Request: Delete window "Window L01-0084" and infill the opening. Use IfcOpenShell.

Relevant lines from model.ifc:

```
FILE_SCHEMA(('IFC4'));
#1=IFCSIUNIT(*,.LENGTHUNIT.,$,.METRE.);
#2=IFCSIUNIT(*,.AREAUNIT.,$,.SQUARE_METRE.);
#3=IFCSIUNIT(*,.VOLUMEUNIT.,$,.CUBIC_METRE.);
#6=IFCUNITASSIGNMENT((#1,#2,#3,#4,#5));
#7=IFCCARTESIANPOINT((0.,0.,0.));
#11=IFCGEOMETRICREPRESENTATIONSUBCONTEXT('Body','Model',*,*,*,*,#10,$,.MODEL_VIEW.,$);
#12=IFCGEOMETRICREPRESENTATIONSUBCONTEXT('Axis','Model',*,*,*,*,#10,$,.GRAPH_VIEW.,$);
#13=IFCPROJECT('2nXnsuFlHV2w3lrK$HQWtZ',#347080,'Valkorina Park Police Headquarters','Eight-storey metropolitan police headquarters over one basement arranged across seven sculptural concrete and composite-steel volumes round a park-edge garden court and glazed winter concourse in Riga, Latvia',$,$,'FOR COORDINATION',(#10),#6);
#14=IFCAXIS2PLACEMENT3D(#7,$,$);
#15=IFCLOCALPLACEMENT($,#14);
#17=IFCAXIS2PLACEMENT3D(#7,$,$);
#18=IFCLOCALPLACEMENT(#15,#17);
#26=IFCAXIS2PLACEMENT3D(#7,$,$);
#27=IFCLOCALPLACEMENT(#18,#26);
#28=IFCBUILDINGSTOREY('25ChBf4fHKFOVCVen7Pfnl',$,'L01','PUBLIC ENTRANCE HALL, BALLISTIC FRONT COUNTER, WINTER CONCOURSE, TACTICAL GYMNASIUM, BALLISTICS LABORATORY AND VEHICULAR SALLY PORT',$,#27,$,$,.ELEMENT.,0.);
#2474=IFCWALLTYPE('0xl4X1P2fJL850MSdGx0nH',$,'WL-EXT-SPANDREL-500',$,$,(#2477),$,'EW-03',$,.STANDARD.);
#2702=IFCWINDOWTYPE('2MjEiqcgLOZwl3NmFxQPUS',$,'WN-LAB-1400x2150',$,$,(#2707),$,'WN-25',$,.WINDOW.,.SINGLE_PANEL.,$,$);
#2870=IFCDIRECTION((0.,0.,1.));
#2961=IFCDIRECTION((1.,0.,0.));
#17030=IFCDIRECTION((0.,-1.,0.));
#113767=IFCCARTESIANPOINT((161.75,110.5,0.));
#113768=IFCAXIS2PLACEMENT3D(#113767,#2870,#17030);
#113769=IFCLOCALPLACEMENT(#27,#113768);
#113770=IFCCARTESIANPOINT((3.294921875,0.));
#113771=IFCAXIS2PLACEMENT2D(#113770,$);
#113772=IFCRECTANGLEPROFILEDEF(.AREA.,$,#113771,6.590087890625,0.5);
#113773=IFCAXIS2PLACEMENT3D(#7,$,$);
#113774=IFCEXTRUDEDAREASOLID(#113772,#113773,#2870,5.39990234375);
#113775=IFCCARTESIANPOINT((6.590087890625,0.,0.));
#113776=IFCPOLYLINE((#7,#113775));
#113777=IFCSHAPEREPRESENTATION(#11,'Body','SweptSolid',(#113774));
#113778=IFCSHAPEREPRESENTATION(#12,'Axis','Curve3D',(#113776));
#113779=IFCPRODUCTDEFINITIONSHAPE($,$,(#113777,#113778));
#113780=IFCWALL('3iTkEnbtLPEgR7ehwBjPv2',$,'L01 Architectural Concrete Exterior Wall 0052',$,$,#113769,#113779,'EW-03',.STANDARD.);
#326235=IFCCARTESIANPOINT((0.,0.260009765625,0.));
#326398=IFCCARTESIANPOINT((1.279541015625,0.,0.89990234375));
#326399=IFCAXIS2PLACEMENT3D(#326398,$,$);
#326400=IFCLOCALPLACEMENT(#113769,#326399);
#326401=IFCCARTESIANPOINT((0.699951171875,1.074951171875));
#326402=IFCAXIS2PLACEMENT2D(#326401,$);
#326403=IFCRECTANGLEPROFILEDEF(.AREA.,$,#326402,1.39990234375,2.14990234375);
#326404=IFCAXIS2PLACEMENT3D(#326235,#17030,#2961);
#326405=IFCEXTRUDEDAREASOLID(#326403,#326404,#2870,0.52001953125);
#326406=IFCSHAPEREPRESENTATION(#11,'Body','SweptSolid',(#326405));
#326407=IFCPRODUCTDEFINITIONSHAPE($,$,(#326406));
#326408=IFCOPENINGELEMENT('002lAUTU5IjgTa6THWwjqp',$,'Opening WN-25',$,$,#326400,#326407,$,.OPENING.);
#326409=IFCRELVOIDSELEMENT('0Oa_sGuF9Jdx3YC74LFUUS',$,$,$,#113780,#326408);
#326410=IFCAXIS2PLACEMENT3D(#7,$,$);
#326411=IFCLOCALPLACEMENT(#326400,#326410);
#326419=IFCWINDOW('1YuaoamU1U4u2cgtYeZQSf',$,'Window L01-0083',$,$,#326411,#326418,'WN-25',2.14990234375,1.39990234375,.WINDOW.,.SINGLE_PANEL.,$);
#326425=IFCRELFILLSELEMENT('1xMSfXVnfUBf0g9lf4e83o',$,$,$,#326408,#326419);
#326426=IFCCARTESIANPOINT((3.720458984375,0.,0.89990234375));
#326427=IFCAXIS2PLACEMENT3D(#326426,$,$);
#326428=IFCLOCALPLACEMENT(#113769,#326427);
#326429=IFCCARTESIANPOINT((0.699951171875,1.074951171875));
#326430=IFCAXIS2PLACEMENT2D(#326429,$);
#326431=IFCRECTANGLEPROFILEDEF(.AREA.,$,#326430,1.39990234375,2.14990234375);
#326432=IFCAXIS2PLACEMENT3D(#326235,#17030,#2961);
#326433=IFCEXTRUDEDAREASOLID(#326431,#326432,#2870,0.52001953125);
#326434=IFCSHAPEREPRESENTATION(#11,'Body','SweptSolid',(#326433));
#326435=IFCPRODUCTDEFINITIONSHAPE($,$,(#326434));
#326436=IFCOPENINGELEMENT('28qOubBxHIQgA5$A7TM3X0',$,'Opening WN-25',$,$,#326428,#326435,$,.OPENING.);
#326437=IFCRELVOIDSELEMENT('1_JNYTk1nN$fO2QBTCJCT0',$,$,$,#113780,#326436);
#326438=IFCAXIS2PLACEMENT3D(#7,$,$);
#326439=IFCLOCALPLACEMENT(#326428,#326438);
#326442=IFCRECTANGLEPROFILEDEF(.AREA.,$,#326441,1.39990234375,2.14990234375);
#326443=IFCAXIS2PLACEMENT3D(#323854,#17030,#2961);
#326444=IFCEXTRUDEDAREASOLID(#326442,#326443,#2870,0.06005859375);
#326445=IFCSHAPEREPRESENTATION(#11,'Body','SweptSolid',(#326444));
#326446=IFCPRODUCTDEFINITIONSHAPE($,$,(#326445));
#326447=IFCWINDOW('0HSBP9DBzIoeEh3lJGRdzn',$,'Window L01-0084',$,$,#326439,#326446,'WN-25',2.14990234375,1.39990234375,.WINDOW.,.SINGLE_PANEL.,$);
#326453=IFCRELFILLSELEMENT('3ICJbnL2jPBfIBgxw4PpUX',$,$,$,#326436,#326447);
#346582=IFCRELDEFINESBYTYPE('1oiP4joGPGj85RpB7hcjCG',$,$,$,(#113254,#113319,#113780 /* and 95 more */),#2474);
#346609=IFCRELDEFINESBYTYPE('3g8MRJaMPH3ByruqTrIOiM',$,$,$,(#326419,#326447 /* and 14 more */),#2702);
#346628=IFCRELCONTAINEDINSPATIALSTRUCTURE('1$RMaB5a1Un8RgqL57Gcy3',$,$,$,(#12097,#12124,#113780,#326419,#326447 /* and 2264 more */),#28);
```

```python
import ifcopenshell
import ifcopenshell.api.feature
import ifcopenshell.api.root
import ifcopenshell.geom
import ifcopenshell.util.shape

model = ifcopenshell.open("model.ifc")
settings = ifcopenshell.geom.settings()


def volume(element):
    """Net volume in cubic metres, openings subtracted."""
    shape = ifcopenshell.geom.create_shape(settings, element)
    return ifcopenshell.util.shape.get_volume(shape.geometry)


window = model.by_guid("0HSBP9DBzIoeEh3lJGRdzn")
opening = window.FillsVoids[0].RelatingOpeningElement
wall = opening.VoidsElements[0].RelatingBuildingElement
before = volume(wall)

ifcopenshell.api.root.remove_product(model, product=window)
ifcopenshell.api.feature.remove_feature(model, feature=opening)

after = volume(wall)

print(f"wall volume {before:.3f} -> {after:.3f} m3")

model.write("model_updated.ifc")
```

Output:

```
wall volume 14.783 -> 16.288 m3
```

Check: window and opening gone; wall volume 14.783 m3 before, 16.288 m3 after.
